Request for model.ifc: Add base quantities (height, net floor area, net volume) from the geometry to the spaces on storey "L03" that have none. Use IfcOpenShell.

First a look at what the model holds.

```python
import ifcopenshell
import ifcopenshell.util.element
import ifcopenshell.util.unit

model = ifcopenshell.open("model.ifc")
print(model.schema)
for unit_type in ("LENGTHUNIT", "AREAUNIT", "VOLUMEUNIT"):
    print(unit_type, ifcopenshell.util.unit.calculate_unit_scale(model, unit_type))
storey = next(s for s in model.by_type("IfcBuildingStorey") if s.Name == "L03")
spaces = [e for e in ifcopenshell.util.element.get_decomposition(storey) if e.is_a("IfcSpace")]
for e in sorted(spaces, key=lambda e: e.id()):
    print(e.id(), e.is_a(), e.Name, list(ifcopenshell.util.element.get_psets(e, qtos_only=True)), sep=" | ")
```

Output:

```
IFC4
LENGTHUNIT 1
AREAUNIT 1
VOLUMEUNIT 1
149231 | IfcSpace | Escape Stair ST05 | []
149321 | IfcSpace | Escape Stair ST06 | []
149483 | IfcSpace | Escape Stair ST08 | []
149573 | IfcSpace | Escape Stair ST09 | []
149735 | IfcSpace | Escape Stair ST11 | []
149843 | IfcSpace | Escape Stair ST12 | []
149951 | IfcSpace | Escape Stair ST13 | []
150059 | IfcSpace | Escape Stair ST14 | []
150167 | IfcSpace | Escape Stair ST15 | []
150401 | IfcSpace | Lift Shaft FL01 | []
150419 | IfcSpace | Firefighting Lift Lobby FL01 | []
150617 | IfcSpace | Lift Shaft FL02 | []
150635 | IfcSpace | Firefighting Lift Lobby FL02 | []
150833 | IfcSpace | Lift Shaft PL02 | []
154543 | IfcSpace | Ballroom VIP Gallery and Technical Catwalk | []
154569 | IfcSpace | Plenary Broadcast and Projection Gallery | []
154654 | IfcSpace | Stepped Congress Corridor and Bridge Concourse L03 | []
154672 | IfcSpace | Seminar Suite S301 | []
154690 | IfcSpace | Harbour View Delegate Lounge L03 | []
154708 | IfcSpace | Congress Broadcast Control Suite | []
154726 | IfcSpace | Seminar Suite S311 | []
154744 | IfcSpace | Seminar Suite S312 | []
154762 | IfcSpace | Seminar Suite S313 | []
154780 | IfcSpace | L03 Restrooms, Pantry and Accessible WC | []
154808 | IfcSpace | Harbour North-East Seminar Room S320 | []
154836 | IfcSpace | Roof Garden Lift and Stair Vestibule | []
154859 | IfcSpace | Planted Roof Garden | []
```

```python
import ifcopenshell
import ifcopenshell.api.pset
import ifcopenshell.geom
import ifcopenshell.util.element
import ifcopenshell.util.shape
import ifcopenshell.util.unit

model = ifcopenshell.open("model.ifc")
unit_scale = ifcopenshell.util.unit.calculate_unit_scale(model)
area_scale = ifcopenshell.util.unit.calculate_unit_scale(model, "AREAUNIT")
volume_scale = ifcopenshell.util.unit.calculate_unit_scale(model, "VOLUMEUNIT")
settings = ifcopenshell.geom.settings()

storey = next(s for s in model.by_type("IfcBuildingStorey") if s.Name == "L03")
spaces = [e for e in ifcopenshell.util.element.get_decomposition(storey) if e.is_a("IfcSpace")]

for e in sorted(spaces, key=lambda e: e.id()):
    if ifcopenshell.util.element.get_psets(e, qtos_only=True, should_inherit=False):
        continue
    # Geometry comes back in metres, in the element's own axes.
    shape = ifcopenshell.geom.create_shape(settings, e)
    values = {
        "Height": ifcopenshell.util.shape.get_z(shape.geometry) / unit_scale,
        "NetFloorArea": ifcopenshell.util.shape.get_footprint_area(shape.geometry) / area_scale,
        "NetVolume": ifcopenshell.util.shape.get_volume(shape.geometry) / volume_scale,
    }
    qto = ifcopenshell.api.pset.add_qto(model, product=e, name="Qto_SpaceBaseQuantities")
    ifcopenshell.api.pset.edit_qto(model, qto=qto, properties=values)
    print(e.id(), {k: round(v, 3) for k, v in values.items()})

model.write("model_rev.ifc")
```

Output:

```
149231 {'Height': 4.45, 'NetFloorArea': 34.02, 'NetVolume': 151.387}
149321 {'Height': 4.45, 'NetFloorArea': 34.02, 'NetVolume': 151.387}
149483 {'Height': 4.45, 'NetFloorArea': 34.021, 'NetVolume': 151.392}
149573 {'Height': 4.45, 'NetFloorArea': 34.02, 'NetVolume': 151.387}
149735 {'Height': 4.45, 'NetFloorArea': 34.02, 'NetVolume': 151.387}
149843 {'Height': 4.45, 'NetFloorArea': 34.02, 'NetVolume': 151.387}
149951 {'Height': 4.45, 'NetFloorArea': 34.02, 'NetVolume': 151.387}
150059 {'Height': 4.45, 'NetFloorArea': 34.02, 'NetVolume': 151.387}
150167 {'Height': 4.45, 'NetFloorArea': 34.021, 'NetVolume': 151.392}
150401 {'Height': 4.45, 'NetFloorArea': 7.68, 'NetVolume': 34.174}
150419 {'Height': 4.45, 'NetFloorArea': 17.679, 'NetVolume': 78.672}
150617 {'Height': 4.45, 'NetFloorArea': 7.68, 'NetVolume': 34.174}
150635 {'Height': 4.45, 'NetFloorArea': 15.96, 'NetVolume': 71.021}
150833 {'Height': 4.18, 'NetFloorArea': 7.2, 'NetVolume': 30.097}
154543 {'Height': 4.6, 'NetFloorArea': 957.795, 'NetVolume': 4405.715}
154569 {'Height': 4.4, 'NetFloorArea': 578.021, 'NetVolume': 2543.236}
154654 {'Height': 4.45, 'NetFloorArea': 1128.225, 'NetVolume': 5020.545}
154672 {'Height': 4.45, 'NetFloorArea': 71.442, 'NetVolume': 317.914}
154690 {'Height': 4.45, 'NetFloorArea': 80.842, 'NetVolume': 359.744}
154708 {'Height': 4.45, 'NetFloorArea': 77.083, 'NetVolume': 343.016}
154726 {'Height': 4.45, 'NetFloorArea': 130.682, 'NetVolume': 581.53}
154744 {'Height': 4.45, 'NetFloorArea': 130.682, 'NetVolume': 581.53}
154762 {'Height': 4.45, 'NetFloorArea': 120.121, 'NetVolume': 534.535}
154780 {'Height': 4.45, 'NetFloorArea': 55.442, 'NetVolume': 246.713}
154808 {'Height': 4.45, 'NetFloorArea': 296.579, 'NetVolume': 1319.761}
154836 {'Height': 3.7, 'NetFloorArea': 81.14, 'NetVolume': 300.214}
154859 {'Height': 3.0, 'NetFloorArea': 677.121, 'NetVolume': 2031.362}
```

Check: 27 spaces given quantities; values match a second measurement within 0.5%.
